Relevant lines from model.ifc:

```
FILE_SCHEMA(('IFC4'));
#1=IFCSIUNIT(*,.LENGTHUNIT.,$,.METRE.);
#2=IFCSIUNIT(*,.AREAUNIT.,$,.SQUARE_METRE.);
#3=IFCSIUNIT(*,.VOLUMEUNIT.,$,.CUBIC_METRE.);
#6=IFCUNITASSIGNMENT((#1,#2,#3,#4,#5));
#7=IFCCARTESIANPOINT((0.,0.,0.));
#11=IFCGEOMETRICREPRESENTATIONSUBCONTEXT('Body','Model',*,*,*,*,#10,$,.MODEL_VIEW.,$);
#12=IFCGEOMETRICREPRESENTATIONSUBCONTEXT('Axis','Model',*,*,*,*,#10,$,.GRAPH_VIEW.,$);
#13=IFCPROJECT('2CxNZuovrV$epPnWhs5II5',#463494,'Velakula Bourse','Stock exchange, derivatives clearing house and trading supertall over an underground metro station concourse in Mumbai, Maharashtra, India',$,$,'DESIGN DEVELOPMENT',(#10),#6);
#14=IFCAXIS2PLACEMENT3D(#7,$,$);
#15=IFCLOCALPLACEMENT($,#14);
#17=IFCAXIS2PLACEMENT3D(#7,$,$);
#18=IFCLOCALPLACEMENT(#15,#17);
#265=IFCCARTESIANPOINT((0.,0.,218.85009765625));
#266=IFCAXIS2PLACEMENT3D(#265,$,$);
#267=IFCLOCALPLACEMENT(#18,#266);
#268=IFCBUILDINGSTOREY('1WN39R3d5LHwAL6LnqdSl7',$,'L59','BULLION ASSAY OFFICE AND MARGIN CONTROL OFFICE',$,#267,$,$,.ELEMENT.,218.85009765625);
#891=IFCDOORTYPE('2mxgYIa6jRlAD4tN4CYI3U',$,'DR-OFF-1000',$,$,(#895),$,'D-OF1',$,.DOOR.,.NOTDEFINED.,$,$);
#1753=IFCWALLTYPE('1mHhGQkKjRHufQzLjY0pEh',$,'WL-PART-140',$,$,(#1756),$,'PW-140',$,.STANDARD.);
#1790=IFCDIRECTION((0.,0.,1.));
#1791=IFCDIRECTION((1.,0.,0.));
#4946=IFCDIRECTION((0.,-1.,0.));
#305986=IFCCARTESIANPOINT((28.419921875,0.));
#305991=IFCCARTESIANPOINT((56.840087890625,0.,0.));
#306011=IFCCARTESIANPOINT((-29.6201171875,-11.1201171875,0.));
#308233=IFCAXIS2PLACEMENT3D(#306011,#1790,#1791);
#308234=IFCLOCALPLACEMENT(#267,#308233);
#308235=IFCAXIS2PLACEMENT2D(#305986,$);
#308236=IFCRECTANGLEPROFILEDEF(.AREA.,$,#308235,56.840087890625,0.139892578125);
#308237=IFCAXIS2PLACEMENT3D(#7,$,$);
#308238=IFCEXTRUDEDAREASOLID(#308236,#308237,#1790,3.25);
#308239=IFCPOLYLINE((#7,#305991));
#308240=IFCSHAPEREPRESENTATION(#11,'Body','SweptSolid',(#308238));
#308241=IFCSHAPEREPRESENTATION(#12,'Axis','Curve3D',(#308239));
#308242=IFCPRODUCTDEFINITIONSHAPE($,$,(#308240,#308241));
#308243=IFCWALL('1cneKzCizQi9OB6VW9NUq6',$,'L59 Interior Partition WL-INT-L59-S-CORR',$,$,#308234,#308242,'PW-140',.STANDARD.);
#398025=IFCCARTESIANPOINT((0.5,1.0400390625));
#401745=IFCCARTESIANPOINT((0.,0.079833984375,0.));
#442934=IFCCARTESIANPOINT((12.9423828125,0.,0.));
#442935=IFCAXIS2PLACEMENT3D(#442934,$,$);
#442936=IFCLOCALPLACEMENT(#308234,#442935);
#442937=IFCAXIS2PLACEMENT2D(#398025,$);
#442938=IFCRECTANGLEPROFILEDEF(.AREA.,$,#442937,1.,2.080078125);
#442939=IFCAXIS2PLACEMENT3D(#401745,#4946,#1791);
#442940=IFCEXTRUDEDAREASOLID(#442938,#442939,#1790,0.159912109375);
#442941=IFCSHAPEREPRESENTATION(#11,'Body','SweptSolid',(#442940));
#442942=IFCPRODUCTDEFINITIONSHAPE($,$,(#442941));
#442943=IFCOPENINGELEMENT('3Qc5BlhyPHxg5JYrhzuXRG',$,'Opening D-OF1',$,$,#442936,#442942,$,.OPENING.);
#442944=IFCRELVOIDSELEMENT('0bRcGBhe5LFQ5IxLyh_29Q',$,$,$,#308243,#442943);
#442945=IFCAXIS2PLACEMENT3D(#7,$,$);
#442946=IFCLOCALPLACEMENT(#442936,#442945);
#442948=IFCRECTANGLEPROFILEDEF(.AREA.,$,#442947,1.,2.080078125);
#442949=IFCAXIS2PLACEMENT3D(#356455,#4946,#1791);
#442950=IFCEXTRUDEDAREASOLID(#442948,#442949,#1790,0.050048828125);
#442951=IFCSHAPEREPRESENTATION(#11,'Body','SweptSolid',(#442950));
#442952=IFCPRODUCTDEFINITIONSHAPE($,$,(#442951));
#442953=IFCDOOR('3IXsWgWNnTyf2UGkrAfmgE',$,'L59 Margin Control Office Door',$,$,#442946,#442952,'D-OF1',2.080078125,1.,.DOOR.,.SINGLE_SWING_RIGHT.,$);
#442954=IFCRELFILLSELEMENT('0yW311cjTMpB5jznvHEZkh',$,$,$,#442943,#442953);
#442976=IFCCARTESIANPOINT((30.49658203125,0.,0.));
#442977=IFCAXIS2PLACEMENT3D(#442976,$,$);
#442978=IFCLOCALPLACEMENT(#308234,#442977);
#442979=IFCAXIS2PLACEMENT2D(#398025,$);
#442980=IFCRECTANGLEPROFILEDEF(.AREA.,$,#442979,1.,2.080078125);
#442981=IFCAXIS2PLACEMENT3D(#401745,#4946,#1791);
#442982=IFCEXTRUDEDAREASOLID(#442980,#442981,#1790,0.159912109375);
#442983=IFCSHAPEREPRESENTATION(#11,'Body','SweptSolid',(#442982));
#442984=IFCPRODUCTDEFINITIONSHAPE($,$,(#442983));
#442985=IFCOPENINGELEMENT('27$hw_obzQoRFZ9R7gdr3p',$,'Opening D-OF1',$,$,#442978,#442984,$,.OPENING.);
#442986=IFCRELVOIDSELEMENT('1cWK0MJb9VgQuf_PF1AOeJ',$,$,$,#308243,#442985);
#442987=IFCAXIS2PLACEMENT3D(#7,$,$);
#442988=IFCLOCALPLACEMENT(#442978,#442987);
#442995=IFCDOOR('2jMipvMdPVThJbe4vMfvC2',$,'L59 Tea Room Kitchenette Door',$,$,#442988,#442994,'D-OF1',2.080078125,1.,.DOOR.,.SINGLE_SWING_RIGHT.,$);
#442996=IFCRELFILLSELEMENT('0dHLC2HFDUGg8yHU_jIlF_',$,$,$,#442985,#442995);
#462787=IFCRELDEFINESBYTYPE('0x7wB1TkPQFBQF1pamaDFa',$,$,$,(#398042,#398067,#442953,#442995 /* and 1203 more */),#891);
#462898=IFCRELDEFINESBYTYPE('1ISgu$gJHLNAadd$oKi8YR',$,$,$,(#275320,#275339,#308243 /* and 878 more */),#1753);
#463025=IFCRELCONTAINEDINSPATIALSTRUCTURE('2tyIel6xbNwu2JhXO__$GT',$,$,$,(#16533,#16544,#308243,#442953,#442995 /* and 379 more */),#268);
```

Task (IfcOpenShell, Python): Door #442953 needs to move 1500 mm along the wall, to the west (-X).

```python
import ifcopenshell
import ifcopenshell.api.geometry
import ifcopenshell.util.placement

model = ifcopenshell.open("model.ifc")

door = model.by_guid("3IXsWgWNnTyf2UGkrAfmgE")
opening = door.FillsVoids[0].RelatingOpeningElement
wall = opening.VoidsElements[0].RelatingBuildingElement

wall_matrix = ifcopenshell.util.placement.get_local_placement(wall.ObjectPlacement)
shift = wall_matrix[:3, 0] * -1.5
before = ifcopenshell.util.placement.get_local_placement(door.ObjectPlacement)[:3, 3].copy()

# The door is placed relative to its opening, so it follows when the opening moves.
matrix = ifcopenshell.util.placement.get_local_placement(opening.ObjectPlacement)
matrix[:3, 3] += shift
ifcopenshell.api.geometry.edit_object_placement(
    model, product=opening, matrix=matrix, is_si=False, should_transform_children=True
)

after = ifcopenshell.util.placement.get_local_placement(door.ObjectPlacement)[:3, 3]
print("door moved by", (after - before).round(3) + 0.0)

model.write("model_edited.ifc")
```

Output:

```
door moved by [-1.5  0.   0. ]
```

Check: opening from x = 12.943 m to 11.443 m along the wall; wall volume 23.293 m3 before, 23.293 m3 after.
